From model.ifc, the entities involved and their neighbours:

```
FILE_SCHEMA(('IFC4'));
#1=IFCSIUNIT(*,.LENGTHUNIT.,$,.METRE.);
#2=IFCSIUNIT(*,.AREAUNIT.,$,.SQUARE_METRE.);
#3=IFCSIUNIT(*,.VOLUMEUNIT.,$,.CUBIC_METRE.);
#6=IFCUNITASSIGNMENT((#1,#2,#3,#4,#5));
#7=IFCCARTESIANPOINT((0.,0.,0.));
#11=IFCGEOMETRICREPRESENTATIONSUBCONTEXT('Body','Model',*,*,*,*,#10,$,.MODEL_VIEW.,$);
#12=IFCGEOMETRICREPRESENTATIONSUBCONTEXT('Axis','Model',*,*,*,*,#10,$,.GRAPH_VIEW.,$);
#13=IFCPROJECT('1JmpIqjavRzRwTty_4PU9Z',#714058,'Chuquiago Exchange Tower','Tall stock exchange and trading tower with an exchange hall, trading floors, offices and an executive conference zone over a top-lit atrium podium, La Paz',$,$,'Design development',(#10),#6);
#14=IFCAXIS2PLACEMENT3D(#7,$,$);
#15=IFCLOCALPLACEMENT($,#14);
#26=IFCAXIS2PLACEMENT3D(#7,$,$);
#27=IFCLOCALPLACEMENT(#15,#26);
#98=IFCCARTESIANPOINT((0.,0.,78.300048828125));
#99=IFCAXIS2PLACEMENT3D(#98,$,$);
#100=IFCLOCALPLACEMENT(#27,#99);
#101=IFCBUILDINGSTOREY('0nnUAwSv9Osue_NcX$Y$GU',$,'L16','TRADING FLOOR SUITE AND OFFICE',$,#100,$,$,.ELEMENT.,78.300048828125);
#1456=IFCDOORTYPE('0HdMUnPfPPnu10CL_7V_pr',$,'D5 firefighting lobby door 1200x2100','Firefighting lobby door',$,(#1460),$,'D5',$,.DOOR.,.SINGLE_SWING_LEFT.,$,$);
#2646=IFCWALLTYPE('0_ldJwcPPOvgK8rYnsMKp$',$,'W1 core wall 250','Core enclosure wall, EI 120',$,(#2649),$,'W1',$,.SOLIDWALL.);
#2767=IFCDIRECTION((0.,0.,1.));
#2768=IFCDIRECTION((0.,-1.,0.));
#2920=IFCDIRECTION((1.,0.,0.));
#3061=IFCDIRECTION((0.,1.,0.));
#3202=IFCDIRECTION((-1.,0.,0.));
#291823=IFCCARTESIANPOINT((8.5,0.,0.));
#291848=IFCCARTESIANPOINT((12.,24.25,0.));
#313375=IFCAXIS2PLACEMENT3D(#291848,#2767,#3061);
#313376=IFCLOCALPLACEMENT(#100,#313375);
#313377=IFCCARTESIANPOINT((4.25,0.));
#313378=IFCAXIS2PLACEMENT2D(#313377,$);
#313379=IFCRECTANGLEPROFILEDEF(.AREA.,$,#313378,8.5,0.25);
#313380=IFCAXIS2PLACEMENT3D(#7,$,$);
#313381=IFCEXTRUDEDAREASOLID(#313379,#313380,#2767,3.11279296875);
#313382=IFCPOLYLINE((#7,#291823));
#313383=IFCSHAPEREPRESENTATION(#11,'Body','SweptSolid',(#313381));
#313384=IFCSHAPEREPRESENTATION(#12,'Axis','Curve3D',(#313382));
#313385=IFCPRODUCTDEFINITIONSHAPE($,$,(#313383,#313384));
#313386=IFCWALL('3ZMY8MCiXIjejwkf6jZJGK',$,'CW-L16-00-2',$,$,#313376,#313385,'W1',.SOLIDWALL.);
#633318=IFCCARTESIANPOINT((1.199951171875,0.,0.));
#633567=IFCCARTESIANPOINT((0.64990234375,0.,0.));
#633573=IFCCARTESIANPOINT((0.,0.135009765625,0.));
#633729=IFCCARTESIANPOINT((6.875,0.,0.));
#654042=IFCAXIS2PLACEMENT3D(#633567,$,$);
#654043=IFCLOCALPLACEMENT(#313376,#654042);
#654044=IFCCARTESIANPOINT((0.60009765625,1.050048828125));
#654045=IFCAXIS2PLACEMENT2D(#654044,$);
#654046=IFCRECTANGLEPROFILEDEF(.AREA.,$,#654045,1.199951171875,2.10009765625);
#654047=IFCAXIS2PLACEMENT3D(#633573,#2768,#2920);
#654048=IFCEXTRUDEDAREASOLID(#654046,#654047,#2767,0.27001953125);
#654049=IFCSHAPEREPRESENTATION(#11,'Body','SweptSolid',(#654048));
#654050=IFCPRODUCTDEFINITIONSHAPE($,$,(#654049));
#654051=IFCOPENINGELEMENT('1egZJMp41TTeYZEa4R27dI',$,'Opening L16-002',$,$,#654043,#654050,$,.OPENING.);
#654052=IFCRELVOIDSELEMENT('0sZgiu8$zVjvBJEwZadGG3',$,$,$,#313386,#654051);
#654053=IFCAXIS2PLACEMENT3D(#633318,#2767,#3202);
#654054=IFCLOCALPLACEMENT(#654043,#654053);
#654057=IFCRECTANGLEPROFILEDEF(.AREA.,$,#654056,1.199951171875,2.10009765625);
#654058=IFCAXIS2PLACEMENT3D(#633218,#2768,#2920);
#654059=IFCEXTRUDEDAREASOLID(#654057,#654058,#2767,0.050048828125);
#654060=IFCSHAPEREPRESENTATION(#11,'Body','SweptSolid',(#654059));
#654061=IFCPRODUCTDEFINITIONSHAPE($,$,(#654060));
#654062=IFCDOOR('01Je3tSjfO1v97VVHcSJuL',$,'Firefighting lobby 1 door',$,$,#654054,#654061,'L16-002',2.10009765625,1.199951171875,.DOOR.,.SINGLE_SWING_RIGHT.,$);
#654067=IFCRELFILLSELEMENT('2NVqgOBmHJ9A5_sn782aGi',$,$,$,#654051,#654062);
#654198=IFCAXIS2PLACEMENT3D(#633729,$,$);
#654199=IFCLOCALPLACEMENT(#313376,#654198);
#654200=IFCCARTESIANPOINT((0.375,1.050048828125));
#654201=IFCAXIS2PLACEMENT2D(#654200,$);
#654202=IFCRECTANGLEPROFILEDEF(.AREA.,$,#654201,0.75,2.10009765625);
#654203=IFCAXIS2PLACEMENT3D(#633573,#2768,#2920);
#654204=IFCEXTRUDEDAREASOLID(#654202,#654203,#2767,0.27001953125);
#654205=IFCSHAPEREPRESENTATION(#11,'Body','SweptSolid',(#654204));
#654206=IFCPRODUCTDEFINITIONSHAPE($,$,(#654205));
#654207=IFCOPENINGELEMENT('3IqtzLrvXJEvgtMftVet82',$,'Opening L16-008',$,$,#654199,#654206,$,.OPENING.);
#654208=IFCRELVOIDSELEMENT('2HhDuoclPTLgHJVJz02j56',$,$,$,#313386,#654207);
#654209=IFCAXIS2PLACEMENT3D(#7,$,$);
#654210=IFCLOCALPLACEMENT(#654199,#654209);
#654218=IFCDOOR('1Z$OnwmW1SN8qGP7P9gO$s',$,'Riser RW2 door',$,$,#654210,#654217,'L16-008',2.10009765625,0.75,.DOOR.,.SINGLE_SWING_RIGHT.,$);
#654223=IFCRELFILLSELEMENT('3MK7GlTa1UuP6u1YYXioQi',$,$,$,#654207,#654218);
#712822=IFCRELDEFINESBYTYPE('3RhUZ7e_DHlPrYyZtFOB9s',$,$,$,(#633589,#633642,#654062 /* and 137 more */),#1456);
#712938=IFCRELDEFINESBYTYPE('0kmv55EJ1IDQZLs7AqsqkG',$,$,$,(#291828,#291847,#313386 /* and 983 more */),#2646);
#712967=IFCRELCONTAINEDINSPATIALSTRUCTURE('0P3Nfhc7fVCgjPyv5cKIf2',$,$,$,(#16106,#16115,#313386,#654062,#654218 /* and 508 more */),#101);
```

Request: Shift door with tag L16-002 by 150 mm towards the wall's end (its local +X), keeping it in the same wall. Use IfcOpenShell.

```python
import ifcopenshell
import ifcopenshell.api.geometry
import ifcopenshell.util.placement

model = ifcopenshell.open("model.ifc")

door = model.by_guid("01Je3tSjfO1v97VVHcSJuL")
opening = door.FillsVoids[0].RelatingOpeningElement
wall = opening.VoidsElements[0].RelatingBuildingElement

wall_matrix = ifcopenshell.util.placement.get_local_placement(wall.ObjectPlacement)
shift = wall_matrix[:3, 0] * 0.15
before = ifcopenshell.util.placement.get_local_placement(door.ObjectPlacement)[:3, 3].copy()

# The door is placed relative to its opening, so it follows when the opening moves.
matrix = ifcopenshell.util.placement.get_local_placement(opening.ObjectPlacement)
matrix[:3, 3] += shift
ifcopenshell.api.geometry.edit_object_placement(
    model, product=opening, matrix=matrix, is_si=False, should_transform_children=True
)

after = ifcopenshell.util.placement.get_local_placement(door.ObjectPlacement)[:3, 3]
print("door moved by", (after - before).round(3) + 0.0)

model.write("model_updated.ifc")
```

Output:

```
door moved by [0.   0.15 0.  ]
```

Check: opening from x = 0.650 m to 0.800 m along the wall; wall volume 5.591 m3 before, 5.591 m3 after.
